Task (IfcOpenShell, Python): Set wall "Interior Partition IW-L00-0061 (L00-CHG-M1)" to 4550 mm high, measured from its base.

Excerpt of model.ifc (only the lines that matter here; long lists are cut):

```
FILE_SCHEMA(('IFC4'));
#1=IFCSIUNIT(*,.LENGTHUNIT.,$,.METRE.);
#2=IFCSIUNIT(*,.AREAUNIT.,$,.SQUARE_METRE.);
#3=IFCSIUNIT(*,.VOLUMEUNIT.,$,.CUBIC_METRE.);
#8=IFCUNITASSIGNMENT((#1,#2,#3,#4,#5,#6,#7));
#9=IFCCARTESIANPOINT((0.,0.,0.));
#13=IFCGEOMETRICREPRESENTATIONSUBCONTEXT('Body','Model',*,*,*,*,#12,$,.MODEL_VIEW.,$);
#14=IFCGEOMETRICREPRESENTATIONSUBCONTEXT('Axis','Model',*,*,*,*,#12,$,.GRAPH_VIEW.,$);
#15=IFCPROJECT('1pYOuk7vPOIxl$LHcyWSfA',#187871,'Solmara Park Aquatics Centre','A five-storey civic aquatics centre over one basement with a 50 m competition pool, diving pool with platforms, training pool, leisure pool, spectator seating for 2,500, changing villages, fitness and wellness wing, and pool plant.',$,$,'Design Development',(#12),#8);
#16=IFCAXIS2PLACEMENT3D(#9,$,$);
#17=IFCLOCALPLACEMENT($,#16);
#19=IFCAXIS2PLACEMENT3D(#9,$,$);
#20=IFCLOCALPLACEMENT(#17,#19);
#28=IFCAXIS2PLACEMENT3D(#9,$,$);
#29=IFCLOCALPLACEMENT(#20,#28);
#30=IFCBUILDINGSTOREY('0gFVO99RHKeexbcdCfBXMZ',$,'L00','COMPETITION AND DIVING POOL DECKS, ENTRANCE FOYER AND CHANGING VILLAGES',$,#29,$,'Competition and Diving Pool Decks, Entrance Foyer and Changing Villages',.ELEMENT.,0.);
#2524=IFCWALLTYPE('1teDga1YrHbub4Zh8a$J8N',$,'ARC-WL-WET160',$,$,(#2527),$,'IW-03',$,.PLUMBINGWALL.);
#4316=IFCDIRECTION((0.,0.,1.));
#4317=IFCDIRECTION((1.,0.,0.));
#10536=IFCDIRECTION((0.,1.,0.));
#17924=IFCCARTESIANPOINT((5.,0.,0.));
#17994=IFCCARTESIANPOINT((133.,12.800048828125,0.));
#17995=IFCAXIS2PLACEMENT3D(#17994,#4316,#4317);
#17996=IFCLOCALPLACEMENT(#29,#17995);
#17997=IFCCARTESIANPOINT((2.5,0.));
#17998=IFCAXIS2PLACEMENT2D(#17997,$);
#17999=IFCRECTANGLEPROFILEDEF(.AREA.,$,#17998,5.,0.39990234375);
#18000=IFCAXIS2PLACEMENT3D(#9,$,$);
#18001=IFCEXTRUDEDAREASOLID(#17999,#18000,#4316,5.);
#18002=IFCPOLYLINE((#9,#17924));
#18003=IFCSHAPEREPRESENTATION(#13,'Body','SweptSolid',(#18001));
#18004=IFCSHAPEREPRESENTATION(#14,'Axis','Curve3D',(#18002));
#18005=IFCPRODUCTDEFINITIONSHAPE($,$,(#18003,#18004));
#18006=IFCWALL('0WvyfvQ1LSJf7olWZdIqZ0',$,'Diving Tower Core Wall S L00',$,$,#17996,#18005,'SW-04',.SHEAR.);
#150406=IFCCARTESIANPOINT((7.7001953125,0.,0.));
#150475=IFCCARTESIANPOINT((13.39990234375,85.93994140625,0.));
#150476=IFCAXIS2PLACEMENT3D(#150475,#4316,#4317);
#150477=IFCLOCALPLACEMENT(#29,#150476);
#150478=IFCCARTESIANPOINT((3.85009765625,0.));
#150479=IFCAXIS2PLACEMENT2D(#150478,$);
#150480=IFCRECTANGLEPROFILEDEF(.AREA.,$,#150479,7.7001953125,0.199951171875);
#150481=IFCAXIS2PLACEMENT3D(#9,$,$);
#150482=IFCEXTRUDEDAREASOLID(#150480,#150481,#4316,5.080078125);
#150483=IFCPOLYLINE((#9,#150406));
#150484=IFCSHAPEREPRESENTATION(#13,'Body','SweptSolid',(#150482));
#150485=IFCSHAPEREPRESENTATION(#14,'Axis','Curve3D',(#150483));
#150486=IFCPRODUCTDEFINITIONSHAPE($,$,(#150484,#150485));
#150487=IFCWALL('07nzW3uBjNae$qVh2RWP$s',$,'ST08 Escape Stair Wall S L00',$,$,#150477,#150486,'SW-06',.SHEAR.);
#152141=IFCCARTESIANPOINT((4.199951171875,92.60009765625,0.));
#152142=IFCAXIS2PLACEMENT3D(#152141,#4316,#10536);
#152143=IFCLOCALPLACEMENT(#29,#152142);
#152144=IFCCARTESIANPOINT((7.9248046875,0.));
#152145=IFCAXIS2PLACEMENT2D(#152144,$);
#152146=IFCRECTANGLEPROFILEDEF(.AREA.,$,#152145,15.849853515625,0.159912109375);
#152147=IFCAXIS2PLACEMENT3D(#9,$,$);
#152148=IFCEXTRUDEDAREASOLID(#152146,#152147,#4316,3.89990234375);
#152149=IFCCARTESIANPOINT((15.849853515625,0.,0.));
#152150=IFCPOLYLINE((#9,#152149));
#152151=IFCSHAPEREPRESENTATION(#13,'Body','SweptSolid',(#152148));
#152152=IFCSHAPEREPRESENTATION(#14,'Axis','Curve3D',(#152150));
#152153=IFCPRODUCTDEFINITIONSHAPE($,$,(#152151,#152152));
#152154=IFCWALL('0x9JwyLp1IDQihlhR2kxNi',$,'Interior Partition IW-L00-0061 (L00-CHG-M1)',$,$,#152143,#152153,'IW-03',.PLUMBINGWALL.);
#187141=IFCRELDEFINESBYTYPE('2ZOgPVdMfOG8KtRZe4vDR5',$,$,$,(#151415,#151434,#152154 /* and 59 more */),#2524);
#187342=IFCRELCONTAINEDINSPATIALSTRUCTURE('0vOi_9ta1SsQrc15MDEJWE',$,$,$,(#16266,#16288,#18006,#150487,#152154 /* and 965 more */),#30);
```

```python
import ifcopenshell
import ifcopenshell.geom
import ifcopenshell.util.representation
import ifcopenshell.util.shape
import ifcopenshell.util.unit

model = ifcopenshell.open("model.ifc")
unit_scale = ifcopenshell.util.unit.calculate_unit_scale(model)
settings = ifcopenshell.geom.settings()


def volume(element):
    """Net volume in cubic metres, openings subtracted."""
    shape = ifcopenshell.geom.create_shape(settings, element)
    return ifcopenshell.util.shape.get_volume(shape.geometry)


wall = model.by_guid("0x9JwyLp1IDQihlhR2kxNi")
before = volume(wall)

body = ifcopenshell.util.representation.get_representation(wall, "Model", "Body")
solid = body.Items[0]
old_height = solid.Depth
solid.Depth = 4.55 / unit_scale
after = volume(wall)

print(f"height {old_height:g} -> {solid.Depth:g}, volume {before:.3f} -> {after:.3f} m3")

model.write("model_rev.ifc")
```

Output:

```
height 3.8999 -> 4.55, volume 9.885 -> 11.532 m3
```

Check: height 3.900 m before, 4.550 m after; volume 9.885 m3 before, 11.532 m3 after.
